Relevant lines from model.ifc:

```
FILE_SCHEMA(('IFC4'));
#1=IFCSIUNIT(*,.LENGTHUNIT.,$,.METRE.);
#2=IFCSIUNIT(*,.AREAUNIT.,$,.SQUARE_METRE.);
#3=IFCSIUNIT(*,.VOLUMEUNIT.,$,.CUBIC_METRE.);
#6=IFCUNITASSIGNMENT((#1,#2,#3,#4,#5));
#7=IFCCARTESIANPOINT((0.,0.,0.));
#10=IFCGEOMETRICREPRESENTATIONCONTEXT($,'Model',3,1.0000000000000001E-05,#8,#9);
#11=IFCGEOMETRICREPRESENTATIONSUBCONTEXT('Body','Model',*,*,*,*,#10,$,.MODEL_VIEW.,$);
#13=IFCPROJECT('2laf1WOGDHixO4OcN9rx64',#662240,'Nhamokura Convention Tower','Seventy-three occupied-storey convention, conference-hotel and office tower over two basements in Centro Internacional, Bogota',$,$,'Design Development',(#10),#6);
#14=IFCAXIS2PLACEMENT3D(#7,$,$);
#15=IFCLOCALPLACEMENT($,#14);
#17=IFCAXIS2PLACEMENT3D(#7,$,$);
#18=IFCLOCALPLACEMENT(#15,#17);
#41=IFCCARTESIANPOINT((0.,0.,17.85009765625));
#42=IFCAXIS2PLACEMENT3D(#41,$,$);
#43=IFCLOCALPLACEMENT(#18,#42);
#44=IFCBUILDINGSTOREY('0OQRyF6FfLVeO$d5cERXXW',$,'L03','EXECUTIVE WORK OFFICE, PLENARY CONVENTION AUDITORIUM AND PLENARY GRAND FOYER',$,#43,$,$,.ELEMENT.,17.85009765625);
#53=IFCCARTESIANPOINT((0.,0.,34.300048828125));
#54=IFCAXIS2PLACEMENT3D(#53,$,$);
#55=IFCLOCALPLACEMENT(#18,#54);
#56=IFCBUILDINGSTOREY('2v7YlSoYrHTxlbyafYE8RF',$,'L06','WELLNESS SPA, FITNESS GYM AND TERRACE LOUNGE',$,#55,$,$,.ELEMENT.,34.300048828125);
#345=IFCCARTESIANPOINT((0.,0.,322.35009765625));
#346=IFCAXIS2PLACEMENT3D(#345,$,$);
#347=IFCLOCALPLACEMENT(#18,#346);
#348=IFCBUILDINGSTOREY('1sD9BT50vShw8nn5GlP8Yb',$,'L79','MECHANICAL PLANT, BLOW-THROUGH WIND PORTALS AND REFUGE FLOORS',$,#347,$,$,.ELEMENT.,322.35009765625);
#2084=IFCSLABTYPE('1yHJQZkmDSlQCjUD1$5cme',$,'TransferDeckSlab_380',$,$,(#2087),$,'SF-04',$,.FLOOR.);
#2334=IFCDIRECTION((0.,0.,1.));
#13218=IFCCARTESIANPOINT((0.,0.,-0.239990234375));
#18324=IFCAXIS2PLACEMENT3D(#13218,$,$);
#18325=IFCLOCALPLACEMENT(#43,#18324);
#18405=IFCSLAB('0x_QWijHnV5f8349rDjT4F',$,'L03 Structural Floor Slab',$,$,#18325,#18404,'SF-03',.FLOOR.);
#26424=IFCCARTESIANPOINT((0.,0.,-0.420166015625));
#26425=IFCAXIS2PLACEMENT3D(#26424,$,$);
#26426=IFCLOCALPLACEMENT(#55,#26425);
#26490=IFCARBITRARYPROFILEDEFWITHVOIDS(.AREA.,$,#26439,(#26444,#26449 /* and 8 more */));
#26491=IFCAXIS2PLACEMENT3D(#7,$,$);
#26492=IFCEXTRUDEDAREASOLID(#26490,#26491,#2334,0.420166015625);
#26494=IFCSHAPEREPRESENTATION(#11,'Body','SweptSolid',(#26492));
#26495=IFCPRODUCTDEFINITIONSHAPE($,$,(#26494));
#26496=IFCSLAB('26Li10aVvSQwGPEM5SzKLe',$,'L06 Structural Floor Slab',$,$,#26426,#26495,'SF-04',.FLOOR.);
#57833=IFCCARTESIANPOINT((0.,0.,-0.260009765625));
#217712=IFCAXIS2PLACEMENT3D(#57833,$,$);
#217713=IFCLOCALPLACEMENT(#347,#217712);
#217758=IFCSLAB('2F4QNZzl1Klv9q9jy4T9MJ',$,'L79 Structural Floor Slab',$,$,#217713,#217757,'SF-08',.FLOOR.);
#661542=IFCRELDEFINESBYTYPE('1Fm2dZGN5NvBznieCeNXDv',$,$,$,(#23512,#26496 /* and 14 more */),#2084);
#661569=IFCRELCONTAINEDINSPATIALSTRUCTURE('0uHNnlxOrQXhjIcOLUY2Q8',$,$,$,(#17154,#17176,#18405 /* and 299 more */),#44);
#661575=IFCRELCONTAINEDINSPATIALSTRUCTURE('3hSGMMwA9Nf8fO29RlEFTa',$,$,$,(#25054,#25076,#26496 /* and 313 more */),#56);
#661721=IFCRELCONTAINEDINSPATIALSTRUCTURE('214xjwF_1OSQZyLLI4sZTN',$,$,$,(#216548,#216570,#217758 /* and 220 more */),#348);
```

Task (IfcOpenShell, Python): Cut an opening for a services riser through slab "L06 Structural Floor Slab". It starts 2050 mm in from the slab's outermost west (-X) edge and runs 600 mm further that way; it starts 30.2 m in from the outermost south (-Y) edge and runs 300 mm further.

```python
import numpy as np
import ifcopenshell
import ifcopenshell.api.feature
import ifcopenshell.api.geometry
import ifcopenshell.api.root
import ifcopenshell.geom
import ifcopenshell.util.placement
import ifcopenshell.util.representation
import ifcopenshell.util.shape
import ifcopenshell.util.unit

model = ifcopenshell.open("model.ifc")
unit_scale = ifcopenshell.util.unit.calculate_unit_scale(model)
settings = ifcopenshell.geom.settings()


def volume(element):
    """Net volume in cubic metres, openings subtracted."""
    shape = ifcopenshell.geom.create_shape(settings, element)
    return ifcopenshell.util.shape.get_volume(shape.geometry)


slab = model.by_id(26496)
before = volume(slab)

# Extent in the slab's own axes, in metres. The edges named are its -X and -Y sides.
slab_shape = ifcopenshell.geom.create_shape(settings, slab)
vertices = ifcopenshell.util.shape.get_vertices(slab_shape.geometry)
x_min, y_min, bottom = vertices.min(axis=0)
top = vertices[:, 2].max()

opening = ifcopenshell.api.root.create_entity(model, ifc_class="IfcOpeningElement", name="Services riser opening", predefined_type="OPENING")
context = ifcopenshell.util.representation.get_context(model, "Model", "Body", "MODEL_VIEW")
width, depth = 0.6, 0.3
outline = [(0.0, 0.0), (width, 0.0), (width, depth), (0.0, depth), (0.0, 0.0)]
# Overshoot both faces by 50 mm so the cut is clean.
shape = ifcopenshell.api.geometry.add_slab_representation(
    model, context=context, depth=top - bottom + 0.1, polyline=outline
)
ifcopenshell.api.geometry.assign_representation(model, product=opening, representation=shape)

matrix = ifcopenshell.util.placement.get_local_placement(slab.ObjectPlacement)
matrix[:, 3] = matrix @ np.append(np.array([x_min + 2.05, y_min + 30.2, bottom - 0.05]) / unit_scale, 1.0)
ifcopenshell.api.geometry.edit_object_placement(model, product=opening, matrix=matrix, is_si=False)
ifcopenshell.api.feature.add_feature(model, feature=opening, element=slab)

after = volume(slab)

print(f"slab volume {before:.3f} -> {after:.3f} m3")

model.write("model_updated.ifc")
```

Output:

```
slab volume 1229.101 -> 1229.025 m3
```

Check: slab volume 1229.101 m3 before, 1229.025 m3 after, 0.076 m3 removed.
